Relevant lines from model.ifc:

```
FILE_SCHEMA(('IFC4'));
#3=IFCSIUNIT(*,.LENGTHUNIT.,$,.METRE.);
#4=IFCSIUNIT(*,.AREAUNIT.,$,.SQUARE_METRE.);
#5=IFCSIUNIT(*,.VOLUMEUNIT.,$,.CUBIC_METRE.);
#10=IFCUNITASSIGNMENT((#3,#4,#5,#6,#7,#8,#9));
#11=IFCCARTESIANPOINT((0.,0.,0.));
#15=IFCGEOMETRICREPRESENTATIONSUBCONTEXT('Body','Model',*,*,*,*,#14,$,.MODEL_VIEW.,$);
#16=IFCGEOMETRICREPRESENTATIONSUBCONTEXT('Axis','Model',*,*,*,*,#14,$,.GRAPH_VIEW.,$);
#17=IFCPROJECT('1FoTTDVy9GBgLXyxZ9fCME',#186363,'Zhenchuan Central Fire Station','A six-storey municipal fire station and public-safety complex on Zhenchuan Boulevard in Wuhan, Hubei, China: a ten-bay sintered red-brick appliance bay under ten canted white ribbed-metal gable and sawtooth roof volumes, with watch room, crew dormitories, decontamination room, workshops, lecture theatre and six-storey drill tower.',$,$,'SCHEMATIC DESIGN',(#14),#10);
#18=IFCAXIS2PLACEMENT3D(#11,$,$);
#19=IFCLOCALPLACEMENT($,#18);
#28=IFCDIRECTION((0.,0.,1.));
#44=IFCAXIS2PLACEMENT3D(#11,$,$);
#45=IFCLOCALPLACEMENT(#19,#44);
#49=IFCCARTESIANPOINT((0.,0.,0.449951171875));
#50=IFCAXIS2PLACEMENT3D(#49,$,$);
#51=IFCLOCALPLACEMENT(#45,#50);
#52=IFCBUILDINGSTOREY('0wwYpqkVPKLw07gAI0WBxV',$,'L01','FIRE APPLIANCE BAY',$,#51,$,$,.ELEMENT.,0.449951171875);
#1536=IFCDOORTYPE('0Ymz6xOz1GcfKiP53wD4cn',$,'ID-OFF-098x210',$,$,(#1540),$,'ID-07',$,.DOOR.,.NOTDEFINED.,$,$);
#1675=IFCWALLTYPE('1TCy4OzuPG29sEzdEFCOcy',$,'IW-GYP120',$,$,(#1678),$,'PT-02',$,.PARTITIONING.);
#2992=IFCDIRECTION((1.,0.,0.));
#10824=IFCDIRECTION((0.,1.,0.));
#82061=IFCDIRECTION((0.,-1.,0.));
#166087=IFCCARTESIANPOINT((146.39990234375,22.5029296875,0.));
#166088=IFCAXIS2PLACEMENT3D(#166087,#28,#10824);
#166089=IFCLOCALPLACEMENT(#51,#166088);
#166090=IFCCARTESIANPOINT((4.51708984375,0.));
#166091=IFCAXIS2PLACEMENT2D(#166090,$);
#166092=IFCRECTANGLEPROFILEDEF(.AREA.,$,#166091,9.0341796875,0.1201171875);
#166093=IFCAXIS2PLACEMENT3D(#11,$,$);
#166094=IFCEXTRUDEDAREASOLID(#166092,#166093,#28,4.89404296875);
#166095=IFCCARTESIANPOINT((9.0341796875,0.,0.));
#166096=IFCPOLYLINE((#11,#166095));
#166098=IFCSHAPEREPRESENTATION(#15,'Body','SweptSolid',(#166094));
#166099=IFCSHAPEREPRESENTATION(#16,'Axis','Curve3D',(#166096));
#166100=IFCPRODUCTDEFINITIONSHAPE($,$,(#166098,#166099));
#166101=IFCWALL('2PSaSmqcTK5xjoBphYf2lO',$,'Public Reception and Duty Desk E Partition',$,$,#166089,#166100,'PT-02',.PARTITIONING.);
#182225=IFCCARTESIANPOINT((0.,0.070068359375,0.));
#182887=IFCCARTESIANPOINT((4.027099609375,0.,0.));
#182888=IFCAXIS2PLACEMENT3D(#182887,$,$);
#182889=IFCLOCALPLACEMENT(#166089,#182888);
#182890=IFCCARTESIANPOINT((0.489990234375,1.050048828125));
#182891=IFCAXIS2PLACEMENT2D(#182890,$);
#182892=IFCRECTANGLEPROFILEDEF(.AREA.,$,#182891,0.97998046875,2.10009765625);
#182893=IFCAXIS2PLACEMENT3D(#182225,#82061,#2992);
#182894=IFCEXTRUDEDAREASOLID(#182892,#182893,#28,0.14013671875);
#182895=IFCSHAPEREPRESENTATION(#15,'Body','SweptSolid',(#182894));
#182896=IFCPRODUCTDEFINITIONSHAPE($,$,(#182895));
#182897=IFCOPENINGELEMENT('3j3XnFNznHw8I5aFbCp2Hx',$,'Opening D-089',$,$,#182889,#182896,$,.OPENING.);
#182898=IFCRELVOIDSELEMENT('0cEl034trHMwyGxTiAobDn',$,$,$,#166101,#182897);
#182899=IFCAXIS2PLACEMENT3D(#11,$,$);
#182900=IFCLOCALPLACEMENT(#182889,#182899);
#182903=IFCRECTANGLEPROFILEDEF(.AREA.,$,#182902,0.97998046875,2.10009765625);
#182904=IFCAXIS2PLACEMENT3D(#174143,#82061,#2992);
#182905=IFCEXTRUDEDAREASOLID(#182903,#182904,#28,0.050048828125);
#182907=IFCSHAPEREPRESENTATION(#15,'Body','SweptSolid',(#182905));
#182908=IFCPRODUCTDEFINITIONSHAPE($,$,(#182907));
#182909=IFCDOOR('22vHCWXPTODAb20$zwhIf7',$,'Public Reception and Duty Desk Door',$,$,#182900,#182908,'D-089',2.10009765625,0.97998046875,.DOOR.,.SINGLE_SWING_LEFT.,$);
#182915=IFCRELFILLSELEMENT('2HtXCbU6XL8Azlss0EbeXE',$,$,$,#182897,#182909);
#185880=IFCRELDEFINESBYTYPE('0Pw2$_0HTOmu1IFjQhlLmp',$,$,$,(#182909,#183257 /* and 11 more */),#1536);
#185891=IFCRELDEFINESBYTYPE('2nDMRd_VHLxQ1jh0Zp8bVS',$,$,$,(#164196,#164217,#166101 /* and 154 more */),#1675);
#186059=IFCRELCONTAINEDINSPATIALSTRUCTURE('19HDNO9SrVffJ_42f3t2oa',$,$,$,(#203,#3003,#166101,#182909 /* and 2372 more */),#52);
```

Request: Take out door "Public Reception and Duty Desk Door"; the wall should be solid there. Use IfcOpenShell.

```python
import ifcopenshell
import ifcopenshell.api.feature
import ifcopenshell.api.root
import ifcopenshell.geom
import ifcopenshell.util.shape

model = ifcopenshell.open("model.ifc")
settings = ifcopenshell.geom.settings()


def volume(element):
    """Net volume in cubic metres, openings subtracted."""
    shape = ifcopenshell.geom.create_shape(settings, element)
    return ifcopenshell.util.shape.get_volume(shape.geometry)


door = model.by_guid("22vHCWXPTODAb20$zwhIf7")
opening = door.FillsVoids[0].RelatingOpeningElement
wall = opening.VoidsElements[0].RelatingBuildingElement
before = volume(wall)

ifcopenshell.api.root.remove_product(model, product=door)
ifcopenshell.api.feature.remove_feature(model, feature=opening)

after = volume(wall)

print(f"wall volume {before:.3f} -> {after:.3f} m3")

model.write("model-out.ifc")
```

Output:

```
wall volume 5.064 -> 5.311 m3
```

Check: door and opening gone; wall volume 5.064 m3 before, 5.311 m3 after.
